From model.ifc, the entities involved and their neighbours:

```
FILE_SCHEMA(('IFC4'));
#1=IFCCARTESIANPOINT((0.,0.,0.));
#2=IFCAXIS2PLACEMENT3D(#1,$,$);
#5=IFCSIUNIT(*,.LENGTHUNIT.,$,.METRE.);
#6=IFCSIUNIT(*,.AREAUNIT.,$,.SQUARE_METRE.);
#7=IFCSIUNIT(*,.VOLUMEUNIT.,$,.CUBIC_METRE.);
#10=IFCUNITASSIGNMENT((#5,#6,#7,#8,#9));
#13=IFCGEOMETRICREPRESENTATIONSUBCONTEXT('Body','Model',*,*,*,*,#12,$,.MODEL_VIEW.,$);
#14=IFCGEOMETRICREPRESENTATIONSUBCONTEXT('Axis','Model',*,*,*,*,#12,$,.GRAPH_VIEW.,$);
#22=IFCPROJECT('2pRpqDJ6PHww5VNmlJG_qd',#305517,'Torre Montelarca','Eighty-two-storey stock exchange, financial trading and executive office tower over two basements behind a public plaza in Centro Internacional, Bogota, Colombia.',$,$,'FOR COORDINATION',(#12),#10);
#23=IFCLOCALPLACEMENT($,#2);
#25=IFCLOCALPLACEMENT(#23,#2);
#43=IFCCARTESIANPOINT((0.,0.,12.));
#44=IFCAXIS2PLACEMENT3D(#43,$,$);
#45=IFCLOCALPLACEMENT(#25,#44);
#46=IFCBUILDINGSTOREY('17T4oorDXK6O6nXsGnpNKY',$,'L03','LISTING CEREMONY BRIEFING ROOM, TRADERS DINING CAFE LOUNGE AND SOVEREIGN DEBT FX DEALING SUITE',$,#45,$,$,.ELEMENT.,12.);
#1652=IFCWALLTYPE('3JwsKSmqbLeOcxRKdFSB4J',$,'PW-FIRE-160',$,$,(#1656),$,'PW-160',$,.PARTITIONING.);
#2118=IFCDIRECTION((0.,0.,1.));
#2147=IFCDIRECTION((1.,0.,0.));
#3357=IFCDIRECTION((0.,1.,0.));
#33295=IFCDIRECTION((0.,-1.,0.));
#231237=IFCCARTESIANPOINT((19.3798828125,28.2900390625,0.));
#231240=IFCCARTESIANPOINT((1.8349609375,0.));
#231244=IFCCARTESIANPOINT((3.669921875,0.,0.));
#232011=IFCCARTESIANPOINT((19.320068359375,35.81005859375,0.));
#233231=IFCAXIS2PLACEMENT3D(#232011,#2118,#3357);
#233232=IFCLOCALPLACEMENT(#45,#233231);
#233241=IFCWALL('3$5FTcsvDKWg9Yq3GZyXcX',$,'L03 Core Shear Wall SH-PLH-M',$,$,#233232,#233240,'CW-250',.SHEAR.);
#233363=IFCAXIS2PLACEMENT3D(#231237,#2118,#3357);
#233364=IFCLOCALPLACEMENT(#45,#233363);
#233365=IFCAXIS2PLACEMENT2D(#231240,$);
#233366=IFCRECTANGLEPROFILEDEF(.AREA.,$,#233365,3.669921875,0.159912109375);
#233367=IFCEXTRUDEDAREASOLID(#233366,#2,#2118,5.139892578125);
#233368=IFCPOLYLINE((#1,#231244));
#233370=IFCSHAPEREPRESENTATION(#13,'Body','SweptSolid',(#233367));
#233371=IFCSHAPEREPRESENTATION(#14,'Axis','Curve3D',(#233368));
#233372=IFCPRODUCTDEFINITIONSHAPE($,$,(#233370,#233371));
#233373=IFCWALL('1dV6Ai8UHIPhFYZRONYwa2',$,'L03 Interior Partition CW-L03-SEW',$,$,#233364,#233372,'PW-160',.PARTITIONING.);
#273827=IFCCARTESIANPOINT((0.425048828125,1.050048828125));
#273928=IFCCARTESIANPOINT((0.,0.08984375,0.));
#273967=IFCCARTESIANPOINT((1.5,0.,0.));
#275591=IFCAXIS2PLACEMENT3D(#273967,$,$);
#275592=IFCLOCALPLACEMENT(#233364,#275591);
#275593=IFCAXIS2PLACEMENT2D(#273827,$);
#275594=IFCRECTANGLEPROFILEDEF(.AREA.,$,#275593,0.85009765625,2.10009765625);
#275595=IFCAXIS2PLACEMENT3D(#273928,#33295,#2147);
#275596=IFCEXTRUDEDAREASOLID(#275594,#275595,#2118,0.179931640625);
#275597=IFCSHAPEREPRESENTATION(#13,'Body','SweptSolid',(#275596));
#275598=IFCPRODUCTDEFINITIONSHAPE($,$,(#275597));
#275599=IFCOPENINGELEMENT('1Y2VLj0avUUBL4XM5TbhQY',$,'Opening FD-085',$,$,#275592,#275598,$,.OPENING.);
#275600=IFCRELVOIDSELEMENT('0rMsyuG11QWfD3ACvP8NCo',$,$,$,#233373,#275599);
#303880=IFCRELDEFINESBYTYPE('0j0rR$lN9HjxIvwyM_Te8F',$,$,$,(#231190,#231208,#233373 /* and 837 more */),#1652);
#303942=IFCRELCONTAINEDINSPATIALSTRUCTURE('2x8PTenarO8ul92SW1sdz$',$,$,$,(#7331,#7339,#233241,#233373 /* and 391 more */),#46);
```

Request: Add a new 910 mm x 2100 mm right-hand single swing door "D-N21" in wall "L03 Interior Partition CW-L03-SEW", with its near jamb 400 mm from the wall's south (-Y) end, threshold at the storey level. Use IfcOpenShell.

```python
import numpy as np
import ifcopenshell
import ifcopenshell.api.feature
import ifcopenshell.api.geometry
import ifcopenshell.api.root
import ifcopenshell.api.spatial
import ifcopenshell.geom
import ifcopenshell.util.element
import ifcopenshell.util.placement
import ifcopenshell.util.representation
import ifcopenshell.util.shape
import ifcopenshell.util.unit

model = ifcopenshell.open("model.ifc")
unit_scale = ifcopenshell.util.unit.calculate_unit_scale(model)
settings = ifcopenshell.geom.settings()


def volume(element):
    """Net volume in cubic metres, openings subtracted."""
    shape = ifcopenshell.geom.create_shape(settings, element)
    return ifcopenshell.util.shape.get_volume(shape.geometry)


wall = model.by_guid("1dV6Ai8UHIPhFYZRONYwa2")
storey = ifcopenshell.util.element.get_container(wall, ifc_class="IfcBuildingStorey")
context = ifcopenshell.util.representation.get_context(model, "Model", "Body", "MODEL_VIEW")
before = volume(wall)

width, height, from_end, sill = 0.91, 2.1, 0.4, 0.0  # metres

# The wall runs along its own X axis, and the end named is its -X end.
wall_shape = ifcopenshell.geom.create_shape(settings, wall)
x, y, z = ifcopenshell.util.shape.get_vertices(wall_shape.geometry).T
start = x.min() + from_end
face, thickness = float(y.min()), float(y.max() - y.min())
wall_matrix = ifcopenshell.util.placement.get_local_placement(wall.ObjectPlacement)
level = ifcopenshell.util.placement.get_local_placement(storey.ObjectPlacement)[2, 3]


def in_wall(x, y):
    """Placement at x, y metres in the wall's axes, at sill height."""
    matrix = wall_matrix.copy()
    matrix[:, 3] = wall_matrix @ np.array([x / unit_scale, y / unit_scale, 0.0, 1.0])
    matrix[2, 3] = level + sill / unit_scale
    return matrix


# Opening: a box that overshoots both wall faces by 50 mm.
opening = ifcopenshell.api.root.create_entity(model, ifc_class="IfcOpeningElement", predefined_type="OPENING")
box = ifcopenshell.api.geometry.add_wall_representation(
    model, context=context, length=width, height=height, thickness=thickness + 0.1
)
ifcopenshell.api.geometry.assign_representation(model, product=opening, representation=box)
ifcopenshell.api.geometry.edit_object_placement(model, product=opening, matrix=in_wall(start, face - 0.05), is_si=False)
ifcopenshell.api.feature.add_feature(model, feature=opening, element=wall)

door = ifcopenshell.api.root.create_entity(model, ifc_class="IfcDoor", name="D-N21", predefined_type="DOOR")
door.OverallWidth, door.OverallHeight = width / unit_scale, height / unit_scale
door.OperationType = "SINGLE_SWING_RIGHT"
body = ifcopenshell.api.geometry.add_door_representation(
    model,
    context=context,
    overall_width=door.OverallWidth,
    overall_height=door.OverallHeight,
    operation_type="SINGLE_SWING_RIGHT",
    lining_properties={"LiningDepth": thickness / unit_scale, "ThresholdDepth": thickness / unit_scale},
)
ifcopenshell.api.geometry.assign_representation(model, product=door, representation=body)
ifcopenshell.api.spatial.assign_container(model, products=[door], relating_structure=storey)
ifcopenshell.api.feature.add_filling(model, opening=opening, element=door)

# The lining spans the wall, so the door starts at the wall face.
ifcopenshell.api.geometry.edit_object_placement(model, product=door, matrix=in_wall(start, face), is_si=False)

after = volume(wall)

print(f"wall volume {before:.3f} -> {after:.3f} m3")

model.write("model_rev.ifc")
```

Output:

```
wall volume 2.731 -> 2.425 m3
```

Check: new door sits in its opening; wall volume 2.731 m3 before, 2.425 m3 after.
